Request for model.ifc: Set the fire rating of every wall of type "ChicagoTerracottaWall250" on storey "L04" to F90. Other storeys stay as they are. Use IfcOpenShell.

First a look at what the model holds.

```python
import ifcopenshell
import ifcopenshell.util.element

model = ifcopenshell.open("model.ifc")
print(model.schema)
storey = next(s for s in model.by_type("IfcBuildingStorey") if s.Name == "L04")
walls = [e for e in ifcopenshell.util.element.get_decomposition(storey) if e.is_a("IfcWall")]
seen = {}
for e in walls:
    element_type = ifcopenshell.util.element.get_type(e)
    key = (element_type.Name if element_type != e and element_type else None, ifcopenshell.util.element.get_pset(e, "Pset_WallCommon", "FireRating"))
    seen[key] = seen.get(key, 0) + 1
for (name, value), count in sorted(seen.items(), key=str):
    print(count, "x", name, "|", value)
```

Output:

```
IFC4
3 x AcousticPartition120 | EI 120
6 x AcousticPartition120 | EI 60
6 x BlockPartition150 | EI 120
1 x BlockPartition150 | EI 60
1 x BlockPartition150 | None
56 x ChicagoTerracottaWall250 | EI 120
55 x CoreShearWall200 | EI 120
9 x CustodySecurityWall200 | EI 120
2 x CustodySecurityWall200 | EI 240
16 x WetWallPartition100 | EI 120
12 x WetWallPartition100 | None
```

```python
import ifcopenshell
import ifcopenshell.api.pset
import ifcopenshell.util.element

model = ifcopenshell.open("model.ifc")

storey = next(s for s in model.by_type("IfcBuildingStorey") if s.Name == "L04")
walls = [e for e in ifcopenshell.util.element.get_decomposition(storey) if e.is_a("IfcWall")]

count = 0
for e in walls:
    element_type = ifcopenshell.util.element.get_type(e)
    if element_type in (None, e) or element_type.Name != "ChicagoTerracottaWall250":
        continue
    # add_pset returns the element's existing set when there is one.
    pset = ifcopenshell.api.pset.add_pset(model, product=e, name="Pset_WallCommon")
    ifcopenshell.api.pset.edit_pset(model, pset=pset, properties={"FireRating": "F90"})
    count += 1

print(count, "walls updated")

model.write("model_updated.ifc")
```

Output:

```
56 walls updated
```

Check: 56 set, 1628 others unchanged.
